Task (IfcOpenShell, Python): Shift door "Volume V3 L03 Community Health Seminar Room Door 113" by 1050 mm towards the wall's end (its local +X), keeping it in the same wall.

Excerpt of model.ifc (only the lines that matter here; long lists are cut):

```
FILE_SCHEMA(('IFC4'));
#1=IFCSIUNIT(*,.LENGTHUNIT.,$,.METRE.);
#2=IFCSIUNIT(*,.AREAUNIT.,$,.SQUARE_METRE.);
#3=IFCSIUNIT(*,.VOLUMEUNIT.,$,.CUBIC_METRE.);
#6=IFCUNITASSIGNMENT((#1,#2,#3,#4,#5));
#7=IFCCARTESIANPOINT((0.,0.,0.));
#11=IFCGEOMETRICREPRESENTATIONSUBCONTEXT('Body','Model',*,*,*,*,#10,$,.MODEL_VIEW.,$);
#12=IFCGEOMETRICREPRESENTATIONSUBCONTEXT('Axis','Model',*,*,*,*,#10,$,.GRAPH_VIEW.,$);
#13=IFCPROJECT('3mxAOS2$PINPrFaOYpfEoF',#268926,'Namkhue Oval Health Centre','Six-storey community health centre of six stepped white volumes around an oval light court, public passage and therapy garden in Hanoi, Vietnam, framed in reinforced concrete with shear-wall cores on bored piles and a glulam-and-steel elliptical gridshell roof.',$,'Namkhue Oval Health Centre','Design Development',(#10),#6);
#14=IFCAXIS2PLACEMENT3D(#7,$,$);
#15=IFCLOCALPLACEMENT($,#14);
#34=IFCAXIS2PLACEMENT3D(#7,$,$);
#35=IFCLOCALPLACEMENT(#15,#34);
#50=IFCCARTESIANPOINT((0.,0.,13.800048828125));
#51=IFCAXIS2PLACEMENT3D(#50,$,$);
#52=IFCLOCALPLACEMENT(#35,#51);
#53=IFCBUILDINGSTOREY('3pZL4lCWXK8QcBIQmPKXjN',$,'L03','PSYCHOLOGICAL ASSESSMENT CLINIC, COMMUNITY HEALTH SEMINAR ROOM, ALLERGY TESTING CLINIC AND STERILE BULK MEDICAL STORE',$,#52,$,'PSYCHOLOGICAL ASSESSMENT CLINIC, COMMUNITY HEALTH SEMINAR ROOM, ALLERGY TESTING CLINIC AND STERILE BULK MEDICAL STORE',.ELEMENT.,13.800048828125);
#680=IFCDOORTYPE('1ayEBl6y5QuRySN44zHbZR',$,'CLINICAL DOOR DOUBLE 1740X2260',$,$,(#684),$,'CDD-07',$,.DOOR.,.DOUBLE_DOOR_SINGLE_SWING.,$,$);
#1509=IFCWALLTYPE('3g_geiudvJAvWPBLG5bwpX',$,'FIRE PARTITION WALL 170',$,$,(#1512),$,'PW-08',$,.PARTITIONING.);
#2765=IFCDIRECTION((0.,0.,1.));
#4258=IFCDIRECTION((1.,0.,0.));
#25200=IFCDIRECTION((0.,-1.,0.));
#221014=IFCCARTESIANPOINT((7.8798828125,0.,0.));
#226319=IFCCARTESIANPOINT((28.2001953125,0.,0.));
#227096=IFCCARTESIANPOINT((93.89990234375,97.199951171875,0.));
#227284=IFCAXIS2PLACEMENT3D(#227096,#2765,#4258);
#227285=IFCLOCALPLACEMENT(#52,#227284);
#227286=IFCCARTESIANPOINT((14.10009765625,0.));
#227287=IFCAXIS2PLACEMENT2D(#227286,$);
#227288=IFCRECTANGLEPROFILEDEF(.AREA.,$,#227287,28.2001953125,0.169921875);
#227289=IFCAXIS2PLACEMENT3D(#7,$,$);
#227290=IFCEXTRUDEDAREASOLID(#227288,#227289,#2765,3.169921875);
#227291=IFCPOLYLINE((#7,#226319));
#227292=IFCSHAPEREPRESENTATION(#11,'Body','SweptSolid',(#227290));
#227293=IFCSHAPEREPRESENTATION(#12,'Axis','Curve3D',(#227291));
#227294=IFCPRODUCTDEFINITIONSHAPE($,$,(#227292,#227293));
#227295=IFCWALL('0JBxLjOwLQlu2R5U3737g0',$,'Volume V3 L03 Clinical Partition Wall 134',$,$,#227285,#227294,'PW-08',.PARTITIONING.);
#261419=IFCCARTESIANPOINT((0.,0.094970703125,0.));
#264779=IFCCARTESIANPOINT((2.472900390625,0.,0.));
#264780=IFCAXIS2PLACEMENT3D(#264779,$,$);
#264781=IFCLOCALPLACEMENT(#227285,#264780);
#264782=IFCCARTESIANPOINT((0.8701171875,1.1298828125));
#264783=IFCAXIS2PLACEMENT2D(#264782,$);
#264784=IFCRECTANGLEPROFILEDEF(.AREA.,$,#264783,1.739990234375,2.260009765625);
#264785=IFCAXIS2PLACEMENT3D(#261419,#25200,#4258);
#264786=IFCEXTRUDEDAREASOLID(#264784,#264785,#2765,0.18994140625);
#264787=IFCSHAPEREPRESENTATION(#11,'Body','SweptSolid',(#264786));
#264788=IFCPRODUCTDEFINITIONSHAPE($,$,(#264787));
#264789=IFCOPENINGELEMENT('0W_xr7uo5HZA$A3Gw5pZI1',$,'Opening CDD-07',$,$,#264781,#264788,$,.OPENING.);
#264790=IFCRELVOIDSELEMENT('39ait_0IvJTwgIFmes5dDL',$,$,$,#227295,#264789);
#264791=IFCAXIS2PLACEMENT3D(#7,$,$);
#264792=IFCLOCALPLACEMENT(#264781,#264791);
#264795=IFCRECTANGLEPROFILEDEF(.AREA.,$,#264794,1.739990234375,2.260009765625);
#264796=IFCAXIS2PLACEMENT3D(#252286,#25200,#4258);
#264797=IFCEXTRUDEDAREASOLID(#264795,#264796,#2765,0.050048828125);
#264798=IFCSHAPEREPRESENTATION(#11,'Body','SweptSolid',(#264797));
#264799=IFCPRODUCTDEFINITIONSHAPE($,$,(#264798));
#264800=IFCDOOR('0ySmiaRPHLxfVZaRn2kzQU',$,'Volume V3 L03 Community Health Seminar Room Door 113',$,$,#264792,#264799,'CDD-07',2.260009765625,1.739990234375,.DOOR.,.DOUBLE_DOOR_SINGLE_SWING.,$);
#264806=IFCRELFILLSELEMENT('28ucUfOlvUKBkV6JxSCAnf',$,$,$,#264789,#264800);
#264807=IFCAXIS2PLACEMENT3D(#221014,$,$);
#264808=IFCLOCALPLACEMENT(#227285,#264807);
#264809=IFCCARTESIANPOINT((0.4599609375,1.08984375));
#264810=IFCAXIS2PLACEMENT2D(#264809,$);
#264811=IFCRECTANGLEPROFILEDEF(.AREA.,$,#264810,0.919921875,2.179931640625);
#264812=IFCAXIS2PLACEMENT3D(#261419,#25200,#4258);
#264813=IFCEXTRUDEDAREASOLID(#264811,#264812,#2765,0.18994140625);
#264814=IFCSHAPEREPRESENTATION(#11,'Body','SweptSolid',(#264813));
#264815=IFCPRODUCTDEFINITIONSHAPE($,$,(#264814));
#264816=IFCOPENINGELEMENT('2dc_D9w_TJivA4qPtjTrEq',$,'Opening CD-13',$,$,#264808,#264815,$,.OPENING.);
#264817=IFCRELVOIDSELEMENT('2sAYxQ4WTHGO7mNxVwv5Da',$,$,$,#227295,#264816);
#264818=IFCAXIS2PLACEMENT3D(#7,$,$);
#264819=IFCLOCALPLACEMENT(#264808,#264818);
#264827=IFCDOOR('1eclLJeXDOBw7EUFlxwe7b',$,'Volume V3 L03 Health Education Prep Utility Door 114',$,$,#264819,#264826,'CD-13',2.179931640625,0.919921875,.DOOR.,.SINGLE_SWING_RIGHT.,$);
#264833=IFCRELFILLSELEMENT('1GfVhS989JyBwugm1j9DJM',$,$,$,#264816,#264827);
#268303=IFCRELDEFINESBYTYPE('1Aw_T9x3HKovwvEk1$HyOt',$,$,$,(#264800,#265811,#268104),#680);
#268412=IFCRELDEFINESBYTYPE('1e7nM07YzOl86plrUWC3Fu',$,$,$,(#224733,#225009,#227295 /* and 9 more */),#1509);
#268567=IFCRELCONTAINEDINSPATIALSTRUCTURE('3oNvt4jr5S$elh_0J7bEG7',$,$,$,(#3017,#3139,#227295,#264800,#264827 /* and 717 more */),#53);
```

```python
import ifcopenshell
import ifcopenshell.api.geometry
import ifcopenshell.util.placement

model = ifcopenshell.open("model.ifc")

door = model.by_guid("0ySmiaRPHLxfVZaRn2kzQU")
opening = door.FillsVoids[0].RelatingOpeningElement
wall = opening.VoidsElements[0].RelatingBuildingElement

wall_matrix = ifcopenshell.util.placement.get_local_placement(wall.ObjectPlacement)
shift = wall_matrix[:3, 0] * 1.05
before = ifcopenshell.util.placement.get_local_placement(door.ObjectPlacement)[:3, 3].copy()

# The door is placed relative to its opening, so it follows when the opening moves.
matrix = ifcopenshell.util.placement.get_local_placement(opening.ObjectPlacement)
matrix[:3, 3] += shift
ifcopenshell.api.geometry.edit_object_placement(
    model, product=opening, matrix=matrix, is_si=False, should_transform_children=True
)

after = ifcopenshell.util.placement.get_local_placement(door.ObjectPlacement)[:3, 3]
print("door moved by", (after - before).round(3) + 0.0)

model.write("model_v2.ifc")
```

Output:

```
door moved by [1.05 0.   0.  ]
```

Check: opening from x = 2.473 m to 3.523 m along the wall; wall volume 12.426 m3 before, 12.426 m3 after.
